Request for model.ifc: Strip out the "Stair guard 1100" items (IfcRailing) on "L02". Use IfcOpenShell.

First a look at what the model holds.

```python
import ifcopenshell
import ifcopenshell.util.element

model = ifcopenshell.open("model.ifc")
print(model.schema)
storey = next(s for s in model.by_type("IfcBuildingStorey") if s.Name == "L02")
railings = [e for e in ifcopenshell.util.element.get_decomposition(storey) if e.is_a("IfcRailing")]
seen = {}
for e in railings:
    element_type = ifcopenshell.util.element.get_type(e)
    name = element_type.Name if element_type not in (None, e) else None
    seen[name] = seen.get(name, 0) + 1
for name, count in sorted(seen.items(), key=str):
    print(count, "x", name)
```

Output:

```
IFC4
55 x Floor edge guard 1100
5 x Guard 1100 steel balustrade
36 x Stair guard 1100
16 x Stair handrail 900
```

```python
import ifcopenshell
import ifcopenshell.api.root
import ifcopenshell.util.element

model = ifcopenshell.open("model.ifc")

storey = next(s for s in model.by_type("IfcBuildingStorey") if s.Name == "L02")
railings = [e for e in ifcopenshell.util.element.get_decomposition(storey) if e.is_a("IfcRailing")]
targets = [e for e in railings if (t := ifcopenshell.util.element.get_type(e)) not in (None, e) and t.Name == "Stair guard 1100"]

for e in targets:
    ifcopenshell.api.root.remove_product(model, product=e)
print(len(targets), "removed")

model.write("model_rev.ifc")
```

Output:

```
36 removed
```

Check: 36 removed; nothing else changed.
